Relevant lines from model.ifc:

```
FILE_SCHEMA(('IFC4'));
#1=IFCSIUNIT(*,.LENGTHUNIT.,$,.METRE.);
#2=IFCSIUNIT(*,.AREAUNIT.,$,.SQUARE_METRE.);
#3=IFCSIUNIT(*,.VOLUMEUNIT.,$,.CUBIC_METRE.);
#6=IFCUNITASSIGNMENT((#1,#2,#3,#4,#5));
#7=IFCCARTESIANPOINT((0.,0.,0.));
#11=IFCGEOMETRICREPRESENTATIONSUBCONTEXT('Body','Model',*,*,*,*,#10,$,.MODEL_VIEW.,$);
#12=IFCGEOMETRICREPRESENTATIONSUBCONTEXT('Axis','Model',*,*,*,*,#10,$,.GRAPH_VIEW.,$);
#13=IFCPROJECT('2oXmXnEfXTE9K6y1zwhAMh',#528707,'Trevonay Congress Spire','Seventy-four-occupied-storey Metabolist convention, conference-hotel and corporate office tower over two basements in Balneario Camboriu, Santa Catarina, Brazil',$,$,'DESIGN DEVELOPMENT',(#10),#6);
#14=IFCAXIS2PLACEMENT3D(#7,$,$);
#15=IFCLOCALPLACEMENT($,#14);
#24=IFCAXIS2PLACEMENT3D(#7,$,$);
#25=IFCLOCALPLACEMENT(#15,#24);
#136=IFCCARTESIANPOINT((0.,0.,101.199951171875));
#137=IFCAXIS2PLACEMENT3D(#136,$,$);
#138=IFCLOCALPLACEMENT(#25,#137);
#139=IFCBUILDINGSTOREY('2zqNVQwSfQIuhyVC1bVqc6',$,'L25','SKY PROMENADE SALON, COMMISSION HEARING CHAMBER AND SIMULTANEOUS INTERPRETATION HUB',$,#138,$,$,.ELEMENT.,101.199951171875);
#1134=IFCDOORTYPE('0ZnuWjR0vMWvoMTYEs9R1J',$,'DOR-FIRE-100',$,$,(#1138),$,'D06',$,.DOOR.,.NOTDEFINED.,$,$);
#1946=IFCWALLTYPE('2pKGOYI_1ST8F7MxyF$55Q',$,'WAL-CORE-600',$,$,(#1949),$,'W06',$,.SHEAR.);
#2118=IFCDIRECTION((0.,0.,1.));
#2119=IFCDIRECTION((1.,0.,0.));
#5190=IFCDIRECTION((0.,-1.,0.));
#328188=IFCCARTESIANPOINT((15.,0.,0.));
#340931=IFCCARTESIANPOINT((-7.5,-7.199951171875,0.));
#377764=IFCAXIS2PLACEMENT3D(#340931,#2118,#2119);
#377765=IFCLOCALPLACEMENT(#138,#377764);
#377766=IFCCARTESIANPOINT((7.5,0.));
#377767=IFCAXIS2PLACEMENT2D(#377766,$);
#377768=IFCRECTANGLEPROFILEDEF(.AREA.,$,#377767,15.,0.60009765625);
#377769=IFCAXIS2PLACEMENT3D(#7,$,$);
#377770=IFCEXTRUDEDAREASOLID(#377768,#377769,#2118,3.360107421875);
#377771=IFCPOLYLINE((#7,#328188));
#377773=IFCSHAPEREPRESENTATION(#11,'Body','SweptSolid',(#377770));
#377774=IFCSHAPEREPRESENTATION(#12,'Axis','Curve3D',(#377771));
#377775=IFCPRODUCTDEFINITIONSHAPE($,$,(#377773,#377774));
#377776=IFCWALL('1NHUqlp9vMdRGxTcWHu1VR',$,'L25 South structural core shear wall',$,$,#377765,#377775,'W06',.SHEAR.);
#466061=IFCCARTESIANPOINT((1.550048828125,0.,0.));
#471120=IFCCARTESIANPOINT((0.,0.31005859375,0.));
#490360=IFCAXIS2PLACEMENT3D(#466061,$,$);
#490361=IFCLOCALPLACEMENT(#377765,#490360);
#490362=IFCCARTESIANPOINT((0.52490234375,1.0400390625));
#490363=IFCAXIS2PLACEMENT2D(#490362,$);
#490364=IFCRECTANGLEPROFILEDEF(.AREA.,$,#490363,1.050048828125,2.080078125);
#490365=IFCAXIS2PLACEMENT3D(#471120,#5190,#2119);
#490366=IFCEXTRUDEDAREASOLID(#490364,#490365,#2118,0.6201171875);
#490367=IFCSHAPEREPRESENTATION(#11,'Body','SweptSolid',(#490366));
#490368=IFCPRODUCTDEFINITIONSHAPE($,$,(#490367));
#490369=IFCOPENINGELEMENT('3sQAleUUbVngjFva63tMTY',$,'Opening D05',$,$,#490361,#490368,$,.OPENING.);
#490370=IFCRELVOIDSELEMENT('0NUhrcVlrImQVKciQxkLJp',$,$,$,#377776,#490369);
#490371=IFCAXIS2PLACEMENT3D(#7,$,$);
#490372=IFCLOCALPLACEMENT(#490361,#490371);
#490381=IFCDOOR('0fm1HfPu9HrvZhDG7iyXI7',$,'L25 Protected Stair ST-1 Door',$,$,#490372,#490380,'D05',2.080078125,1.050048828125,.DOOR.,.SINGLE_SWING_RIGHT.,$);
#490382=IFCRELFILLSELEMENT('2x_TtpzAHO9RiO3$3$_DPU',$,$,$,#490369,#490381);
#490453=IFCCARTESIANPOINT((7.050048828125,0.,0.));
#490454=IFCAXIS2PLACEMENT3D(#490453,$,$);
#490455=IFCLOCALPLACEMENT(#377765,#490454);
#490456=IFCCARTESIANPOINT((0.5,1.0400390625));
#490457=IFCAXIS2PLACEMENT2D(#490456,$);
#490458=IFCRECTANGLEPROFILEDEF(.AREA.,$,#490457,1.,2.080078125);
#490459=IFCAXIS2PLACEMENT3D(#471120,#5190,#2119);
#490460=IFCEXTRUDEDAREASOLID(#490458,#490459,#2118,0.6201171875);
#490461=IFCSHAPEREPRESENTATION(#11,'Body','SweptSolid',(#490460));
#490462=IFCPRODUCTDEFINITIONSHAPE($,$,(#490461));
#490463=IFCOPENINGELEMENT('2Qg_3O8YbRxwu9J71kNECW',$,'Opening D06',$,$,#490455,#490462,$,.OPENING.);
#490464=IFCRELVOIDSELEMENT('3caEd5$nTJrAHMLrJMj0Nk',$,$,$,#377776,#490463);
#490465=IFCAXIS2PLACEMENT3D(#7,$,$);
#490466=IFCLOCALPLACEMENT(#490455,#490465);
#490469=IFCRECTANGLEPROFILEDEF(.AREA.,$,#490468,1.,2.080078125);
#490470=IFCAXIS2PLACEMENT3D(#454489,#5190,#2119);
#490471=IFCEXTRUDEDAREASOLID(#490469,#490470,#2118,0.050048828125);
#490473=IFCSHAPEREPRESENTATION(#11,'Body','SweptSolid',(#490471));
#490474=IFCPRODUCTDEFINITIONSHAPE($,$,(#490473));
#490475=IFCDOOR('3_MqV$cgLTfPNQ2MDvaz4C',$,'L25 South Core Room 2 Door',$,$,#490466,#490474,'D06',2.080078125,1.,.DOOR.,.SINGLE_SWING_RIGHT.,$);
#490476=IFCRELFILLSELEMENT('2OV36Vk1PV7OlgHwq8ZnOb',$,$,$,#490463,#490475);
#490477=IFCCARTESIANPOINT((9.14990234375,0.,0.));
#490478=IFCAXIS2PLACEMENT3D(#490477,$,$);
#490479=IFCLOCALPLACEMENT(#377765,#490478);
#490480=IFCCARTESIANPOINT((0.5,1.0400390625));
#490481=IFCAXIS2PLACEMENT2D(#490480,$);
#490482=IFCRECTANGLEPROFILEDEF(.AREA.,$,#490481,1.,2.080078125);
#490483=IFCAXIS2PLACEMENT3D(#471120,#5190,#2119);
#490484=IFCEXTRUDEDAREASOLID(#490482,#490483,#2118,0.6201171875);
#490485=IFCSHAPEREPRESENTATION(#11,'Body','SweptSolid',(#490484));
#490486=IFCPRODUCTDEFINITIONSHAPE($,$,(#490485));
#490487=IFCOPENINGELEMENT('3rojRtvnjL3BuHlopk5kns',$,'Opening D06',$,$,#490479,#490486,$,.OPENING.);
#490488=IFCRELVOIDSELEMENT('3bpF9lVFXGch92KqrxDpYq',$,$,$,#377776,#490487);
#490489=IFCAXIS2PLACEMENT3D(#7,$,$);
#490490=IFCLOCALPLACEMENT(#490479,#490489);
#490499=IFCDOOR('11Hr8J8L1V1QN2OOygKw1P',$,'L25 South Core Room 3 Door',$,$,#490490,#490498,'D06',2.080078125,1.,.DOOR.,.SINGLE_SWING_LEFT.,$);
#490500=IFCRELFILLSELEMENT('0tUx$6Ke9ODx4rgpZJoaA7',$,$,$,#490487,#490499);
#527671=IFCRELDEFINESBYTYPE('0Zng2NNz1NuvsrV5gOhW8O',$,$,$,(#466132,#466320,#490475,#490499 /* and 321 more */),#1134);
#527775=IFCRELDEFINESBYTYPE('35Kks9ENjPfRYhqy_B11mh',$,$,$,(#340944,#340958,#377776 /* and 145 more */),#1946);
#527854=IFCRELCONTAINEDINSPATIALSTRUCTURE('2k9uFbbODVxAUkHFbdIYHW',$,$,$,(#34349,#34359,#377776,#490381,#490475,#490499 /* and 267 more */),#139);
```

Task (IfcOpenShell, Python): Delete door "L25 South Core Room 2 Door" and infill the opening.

```python
import ifcopenshell
import ifcopenshell.api.feature
import ifcopenshell.api.root
import ifcopenshell.geom
import ifcopenshell.util.shape

model = ifcopenshell.open("model.ifc")
settings = ifcopenshell.geom.settings()


def volume(element):
    """Net volume in cubic metres, openings subtracted."""
    shape = ifcopenshell.geom.create_shape(settings, element)
    return ifcopenshell.util.shape.get_volume(shape.geometry)


door = model.by_guid("3_MqV$cgLTfPNQ2MDvaz4C")
opening = door.FillsVoids[0].RelatingOpeningElement
wall = opening.VoidsElements[0].RelatingBuildingElement
before = volume(wall)

ifcopenshell.api.root.remove_product(model, product=door)
ifcopenshell.api.feature.remove_feature(model, feature=opening)

after = volume(wall)

print(f"wall volume {before:.3f} -> {after:.3f} m3")

model.write("model_edited.ifc")
```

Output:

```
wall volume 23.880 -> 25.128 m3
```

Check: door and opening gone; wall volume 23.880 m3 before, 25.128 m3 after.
